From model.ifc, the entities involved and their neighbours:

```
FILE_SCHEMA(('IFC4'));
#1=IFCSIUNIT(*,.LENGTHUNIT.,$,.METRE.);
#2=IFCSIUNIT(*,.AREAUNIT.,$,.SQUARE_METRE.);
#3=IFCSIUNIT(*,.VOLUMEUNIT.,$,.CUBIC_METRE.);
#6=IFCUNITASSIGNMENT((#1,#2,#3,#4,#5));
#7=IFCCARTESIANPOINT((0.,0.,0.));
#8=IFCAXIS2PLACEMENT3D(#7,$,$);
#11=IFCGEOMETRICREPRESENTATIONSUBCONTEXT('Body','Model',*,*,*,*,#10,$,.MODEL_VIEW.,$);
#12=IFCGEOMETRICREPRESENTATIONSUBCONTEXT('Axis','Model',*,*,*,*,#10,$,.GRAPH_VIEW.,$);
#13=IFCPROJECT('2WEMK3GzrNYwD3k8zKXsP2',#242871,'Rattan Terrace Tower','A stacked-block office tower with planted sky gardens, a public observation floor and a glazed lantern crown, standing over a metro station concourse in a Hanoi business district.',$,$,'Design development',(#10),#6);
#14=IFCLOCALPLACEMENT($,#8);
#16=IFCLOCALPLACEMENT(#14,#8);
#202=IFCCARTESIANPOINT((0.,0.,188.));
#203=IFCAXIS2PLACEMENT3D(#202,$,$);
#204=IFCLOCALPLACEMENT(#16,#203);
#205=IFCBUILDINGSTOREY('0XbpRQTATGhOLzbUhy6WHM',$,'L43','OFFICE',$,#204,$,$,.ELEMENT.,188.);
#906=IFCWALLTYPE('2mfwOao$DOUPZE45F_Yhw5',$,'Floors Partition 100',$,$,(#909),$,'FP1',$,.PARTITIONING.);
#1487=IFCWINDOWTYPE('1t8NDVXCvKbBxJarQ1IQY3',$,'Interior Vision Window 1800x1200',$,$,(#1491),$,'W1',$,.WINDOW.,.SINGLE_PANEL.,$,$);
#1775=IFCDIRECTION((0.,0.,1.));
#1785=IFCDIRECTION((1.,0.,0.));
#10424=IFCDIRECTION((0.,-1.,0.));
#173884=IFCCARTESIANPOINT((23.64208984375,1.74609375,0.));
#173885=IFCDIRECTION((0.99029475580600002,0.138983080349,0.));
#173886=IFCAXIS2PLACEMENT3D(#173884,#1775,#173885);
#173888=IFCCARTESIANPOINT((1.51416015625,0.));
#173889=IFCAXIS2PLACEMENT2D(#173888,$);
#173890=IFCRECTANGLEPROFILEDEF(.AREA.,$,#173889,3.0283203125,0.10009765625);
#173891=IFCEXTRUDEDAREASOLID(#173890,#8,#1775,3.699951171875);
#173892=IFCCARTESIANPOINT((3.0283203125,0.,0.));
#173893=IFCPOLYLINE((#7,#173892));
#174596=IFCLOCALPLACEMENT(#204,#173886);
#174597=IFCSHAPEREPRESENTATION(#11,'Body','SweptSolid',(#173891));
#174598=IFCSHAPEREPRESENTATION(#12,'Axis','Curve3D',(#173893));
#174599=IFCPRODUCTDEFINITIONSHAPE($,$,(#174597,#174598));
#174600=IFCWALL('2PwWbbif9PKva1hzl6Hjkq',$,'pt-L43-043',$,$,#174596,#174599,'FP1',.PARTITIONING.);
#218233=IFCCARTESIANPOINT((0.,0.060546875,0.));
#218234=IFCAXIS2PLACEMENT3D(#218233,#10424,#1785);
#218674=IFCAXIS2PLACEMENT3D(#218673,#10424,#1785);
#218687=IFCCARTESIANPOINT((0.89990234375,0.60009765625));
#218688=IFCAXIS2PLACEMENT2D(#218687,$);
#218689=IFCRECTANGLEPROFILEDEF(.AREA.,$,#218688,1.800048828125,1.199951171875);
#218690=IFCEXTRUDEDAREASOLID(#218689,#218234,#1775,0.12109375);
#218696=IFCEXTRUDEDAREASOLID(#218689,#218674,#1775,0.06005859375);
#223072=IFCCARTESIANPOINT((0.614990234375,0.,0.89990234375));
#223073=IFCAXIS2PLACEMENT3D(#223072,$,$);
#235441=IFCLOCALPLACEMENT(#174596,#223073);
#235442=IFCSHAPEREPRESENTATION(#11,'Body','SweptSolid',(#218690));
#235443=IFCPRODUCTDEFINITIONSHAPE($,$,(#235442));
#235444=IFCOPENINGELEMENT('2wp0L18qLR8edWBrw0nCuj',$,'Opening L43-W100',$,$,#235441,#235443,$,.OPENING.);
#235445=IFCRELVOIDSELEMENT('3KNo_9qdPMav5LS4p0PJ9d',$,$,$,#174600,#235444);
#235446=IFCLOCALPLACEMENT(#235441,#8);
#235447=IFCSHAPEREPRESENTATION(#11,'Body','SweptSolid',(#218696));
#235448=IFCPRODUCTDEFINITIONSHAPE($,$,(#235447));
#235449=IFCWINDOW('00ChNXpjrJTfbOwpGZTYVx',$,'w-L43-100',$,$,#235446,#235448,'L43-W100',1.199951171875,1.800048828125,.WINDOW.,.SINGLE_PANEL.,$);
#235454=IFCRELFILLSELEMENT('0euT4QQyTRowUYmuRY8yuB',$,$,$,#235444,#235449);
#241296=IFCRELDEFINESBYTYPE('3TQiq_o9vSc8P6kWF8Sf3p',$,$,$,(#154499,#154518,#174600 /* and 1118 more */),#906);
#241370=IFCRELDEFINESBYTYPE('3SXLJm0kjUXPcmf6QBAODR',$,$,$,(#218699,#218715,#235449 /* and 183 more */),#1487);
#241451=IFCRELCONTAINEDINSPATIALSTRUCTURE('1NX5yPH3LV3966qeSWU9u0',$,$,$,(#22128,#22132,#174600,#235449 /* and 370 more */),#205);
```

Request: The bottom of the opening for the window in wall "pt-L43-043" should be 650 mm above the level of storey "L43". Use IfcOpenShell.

```python
import numpy as np
import ifcopenshell
import ifcopenshell.api.geometry
import ifcopenshell.geom
import ifcopenshell.util.element
import ifcopenshell.util.placement
import ifcopenshell.util.shape
import ifcopenshell.util.unit

model = ifcopenshell.open("model.ifc")
unit_scale = ifcopenshell.util.unit.calculate_unit_scale(model)

window = model.by_id(235449)
opening = window.FillsVoids[0].RelatingOpeningElement
storey = ifcopenshell.util.element.get_container(window, ifc_class="IfcBuildingStorey")
level = ifcopenshell.util.placement.get_local_placement(storey.ObjectPlacement)[2, 3]

# The opening's origin need not be at the sill, so measure its lowest point.
shape = ifcopenshell.geom.create_shape(ifcopenshell.geom.settings(), opening)
bottom = ifcopenshell.util.shape.get_shape_bottom_elevation(shape, shape.geometry) / unit_scale
dz = level + 0.65 / unit_scale - bottom

shift = np.array([0.0, 0.0, dz])
# The window is placed relative to its opening, so it follows when the opening moves.
matrix = ifcopenshell.util.placement.get_local_placement(opening.ObjectPlacement)
matrix[:3, 3] += shift
ifcopenshell.api.geometry.edit_object_placement(
    model, product=opening, matrix=matrix, is_si=False, should_transform_children=True
)

print(f"moved by {dz * unit_scale:+.3f} m")

model.write("model_v2.ifc")
```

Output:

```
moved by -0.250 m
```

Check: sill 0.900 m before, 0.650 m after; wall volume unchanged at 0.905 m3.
